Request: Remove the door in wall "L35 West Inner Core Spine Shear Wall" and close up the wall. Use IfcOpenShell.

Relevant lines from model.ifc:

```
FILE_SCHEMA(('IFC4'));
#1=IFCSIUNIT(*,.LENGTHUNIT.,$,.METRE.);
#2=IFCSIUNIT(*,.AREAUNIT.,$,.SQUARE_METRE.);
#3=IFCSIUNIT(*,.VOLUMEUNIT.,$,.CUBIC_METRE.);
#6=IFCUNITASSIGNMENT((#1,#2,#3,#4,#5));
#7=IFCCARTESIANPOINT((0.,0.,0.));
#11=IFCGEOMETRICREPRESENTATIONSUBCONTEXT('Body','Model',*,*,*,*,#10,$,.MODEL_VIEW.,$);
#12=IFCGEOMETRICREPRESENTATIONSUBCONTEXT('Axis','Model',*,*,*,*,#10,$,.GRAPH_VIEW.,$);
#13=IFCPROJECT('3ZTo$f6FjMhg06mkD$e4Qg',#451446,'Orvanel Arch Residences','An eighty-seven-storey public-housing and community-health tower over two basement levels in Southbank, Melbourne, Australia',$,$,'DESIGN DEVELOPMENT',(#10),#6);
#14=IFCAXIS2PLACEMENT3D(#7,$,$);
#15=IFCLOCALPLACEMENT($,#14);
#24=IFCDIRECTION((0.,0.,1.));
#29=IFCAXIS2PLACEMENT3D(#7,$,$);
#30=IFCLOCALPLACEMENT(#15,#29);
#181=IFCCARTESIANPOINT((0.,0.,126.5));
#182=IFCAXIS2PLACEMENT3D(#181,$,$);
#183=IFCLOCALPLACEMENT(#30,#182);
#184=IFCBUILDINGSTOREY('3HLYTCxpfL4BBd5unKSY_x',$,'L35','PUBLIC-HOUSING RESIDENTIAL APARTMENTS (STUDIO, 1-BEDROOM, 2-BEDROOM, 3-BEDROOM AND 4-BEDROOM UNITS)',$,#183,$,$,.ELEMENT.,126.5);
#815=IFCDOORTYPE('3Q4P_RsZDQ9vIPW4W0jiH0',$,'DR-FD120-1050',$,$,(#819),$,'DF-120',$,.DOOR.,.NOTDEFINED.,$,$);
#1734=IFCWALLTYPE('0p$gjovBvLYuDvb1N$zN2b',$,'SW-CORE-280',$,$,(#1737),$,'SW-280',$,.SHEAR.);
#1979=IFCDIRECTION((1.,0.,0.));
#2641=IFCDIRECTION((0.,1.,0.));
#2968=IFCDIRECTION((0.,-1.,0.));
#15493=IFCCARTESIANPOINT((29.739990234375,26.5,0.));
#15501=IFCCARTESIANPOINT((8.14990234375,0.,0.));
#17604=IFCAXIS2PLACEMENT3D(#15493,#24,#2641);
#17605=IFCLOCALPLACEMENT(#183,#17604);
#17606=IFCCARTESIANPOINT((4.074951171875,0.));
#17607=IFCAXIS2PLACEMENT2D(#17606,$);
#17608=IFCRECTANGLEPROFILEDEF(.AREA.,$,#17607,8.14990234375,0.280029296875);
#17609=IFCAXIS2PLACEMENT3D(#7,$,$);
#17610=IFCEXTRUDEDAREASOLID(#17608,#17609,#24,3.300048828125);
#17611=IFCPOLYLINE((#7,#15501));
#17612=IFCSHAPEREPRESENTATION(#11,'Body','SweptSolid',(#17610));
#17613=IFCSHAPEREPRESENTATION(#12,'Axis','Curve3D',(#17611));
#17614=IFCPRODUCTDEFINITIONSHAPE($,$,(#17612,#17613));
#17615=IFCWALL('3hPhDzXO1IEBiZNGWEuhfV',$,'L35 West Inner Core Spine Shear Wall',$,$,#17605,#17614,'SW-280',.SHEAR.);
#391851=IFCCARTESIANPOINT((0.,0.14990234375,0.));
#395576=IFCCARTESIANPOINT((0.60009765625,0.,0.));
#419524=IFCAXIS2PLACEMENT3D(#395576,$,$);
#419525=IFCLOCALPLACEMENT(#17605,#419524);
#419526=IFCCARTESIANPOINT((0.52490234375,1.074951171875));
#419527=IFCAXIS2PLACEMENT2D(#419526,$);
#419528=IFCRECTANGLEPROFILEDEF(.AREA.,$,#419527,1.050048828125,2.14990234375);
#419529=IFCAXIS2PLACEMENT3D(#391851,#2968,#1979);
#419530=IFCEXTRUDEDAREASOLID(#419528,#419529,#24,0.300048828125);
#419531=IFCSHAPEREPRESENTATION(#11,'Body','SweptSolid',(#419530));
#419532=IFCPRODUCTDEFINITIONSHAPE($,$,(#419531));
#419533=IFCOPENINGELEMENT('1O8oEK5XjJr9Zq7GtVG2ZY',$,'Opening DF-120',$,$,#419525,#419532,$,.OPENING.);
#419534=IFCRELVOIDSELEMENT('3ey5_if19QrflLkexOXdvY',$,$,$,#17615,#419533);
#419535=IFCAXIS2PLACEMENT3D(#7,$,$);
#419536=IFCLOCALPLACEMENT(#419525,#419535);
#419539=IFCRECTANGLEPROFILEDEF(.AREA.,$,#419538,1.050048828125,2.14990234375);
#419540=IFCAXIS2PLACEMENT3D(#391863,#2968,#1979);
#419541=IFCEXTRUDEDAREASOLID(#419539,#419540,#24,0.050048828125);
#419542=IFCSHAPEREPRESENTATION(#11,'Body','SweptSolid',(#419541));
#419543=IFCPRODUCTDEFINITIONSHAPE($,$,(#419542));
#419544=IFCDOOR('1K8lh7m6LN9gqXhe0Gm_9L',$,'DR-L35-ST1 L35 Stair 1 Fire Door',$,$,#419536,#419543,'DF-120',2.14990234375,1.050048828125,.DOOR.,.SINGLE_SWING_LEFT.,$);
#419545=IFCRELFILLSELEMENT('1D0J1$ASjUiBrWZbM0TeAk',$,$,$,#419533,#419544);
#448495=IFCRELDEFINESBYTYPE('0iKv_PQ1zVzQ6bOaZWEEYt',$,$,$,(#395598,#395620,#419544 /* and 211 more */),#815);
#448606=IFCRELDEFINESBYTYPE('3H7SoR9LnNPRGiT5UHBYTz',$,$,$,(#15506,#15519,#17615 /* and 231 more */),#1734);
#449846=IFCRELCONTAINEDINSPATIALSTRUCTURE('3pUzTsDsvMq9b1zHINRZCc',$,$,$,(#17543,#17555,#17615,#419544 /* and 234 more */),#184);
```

```python
import ifcopenshell
import ifcopenshell.api.feature
import ifcopenshell.api.root
import ifcopenshell.geom
import ifcopenshell.util.shape

model = ifcopenshell.open("model.ifc")
settings = ifcopenshell.geom.settings()


def volume(element):
    """Net volume in cubic metres, openings subtracted."""
    shape = ifcopenshell.geom.create_shape(settings, element)
    return ifcopenshell.util.shape.get_volume(shape.geometry)


door = model.by_id(419544)
opening = door.FillsVoids[0].RelatingOpeningElement
wall = opening.VoidsElements[0].RelatingBuildingElement
before = volume(wall)

ifcopenshell.api.root.remove_product(model, product=door)
ifcopenshell.api.feature.remove_feature(model, feature=opening)

after = volume(wall)

print(f"wall volume {before:.3f} -> {after:.3f} m3")

model.write("model-out.ifc")
```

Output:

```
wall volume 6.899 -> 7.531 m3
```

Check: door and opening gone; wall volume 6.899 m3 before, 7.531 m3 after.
